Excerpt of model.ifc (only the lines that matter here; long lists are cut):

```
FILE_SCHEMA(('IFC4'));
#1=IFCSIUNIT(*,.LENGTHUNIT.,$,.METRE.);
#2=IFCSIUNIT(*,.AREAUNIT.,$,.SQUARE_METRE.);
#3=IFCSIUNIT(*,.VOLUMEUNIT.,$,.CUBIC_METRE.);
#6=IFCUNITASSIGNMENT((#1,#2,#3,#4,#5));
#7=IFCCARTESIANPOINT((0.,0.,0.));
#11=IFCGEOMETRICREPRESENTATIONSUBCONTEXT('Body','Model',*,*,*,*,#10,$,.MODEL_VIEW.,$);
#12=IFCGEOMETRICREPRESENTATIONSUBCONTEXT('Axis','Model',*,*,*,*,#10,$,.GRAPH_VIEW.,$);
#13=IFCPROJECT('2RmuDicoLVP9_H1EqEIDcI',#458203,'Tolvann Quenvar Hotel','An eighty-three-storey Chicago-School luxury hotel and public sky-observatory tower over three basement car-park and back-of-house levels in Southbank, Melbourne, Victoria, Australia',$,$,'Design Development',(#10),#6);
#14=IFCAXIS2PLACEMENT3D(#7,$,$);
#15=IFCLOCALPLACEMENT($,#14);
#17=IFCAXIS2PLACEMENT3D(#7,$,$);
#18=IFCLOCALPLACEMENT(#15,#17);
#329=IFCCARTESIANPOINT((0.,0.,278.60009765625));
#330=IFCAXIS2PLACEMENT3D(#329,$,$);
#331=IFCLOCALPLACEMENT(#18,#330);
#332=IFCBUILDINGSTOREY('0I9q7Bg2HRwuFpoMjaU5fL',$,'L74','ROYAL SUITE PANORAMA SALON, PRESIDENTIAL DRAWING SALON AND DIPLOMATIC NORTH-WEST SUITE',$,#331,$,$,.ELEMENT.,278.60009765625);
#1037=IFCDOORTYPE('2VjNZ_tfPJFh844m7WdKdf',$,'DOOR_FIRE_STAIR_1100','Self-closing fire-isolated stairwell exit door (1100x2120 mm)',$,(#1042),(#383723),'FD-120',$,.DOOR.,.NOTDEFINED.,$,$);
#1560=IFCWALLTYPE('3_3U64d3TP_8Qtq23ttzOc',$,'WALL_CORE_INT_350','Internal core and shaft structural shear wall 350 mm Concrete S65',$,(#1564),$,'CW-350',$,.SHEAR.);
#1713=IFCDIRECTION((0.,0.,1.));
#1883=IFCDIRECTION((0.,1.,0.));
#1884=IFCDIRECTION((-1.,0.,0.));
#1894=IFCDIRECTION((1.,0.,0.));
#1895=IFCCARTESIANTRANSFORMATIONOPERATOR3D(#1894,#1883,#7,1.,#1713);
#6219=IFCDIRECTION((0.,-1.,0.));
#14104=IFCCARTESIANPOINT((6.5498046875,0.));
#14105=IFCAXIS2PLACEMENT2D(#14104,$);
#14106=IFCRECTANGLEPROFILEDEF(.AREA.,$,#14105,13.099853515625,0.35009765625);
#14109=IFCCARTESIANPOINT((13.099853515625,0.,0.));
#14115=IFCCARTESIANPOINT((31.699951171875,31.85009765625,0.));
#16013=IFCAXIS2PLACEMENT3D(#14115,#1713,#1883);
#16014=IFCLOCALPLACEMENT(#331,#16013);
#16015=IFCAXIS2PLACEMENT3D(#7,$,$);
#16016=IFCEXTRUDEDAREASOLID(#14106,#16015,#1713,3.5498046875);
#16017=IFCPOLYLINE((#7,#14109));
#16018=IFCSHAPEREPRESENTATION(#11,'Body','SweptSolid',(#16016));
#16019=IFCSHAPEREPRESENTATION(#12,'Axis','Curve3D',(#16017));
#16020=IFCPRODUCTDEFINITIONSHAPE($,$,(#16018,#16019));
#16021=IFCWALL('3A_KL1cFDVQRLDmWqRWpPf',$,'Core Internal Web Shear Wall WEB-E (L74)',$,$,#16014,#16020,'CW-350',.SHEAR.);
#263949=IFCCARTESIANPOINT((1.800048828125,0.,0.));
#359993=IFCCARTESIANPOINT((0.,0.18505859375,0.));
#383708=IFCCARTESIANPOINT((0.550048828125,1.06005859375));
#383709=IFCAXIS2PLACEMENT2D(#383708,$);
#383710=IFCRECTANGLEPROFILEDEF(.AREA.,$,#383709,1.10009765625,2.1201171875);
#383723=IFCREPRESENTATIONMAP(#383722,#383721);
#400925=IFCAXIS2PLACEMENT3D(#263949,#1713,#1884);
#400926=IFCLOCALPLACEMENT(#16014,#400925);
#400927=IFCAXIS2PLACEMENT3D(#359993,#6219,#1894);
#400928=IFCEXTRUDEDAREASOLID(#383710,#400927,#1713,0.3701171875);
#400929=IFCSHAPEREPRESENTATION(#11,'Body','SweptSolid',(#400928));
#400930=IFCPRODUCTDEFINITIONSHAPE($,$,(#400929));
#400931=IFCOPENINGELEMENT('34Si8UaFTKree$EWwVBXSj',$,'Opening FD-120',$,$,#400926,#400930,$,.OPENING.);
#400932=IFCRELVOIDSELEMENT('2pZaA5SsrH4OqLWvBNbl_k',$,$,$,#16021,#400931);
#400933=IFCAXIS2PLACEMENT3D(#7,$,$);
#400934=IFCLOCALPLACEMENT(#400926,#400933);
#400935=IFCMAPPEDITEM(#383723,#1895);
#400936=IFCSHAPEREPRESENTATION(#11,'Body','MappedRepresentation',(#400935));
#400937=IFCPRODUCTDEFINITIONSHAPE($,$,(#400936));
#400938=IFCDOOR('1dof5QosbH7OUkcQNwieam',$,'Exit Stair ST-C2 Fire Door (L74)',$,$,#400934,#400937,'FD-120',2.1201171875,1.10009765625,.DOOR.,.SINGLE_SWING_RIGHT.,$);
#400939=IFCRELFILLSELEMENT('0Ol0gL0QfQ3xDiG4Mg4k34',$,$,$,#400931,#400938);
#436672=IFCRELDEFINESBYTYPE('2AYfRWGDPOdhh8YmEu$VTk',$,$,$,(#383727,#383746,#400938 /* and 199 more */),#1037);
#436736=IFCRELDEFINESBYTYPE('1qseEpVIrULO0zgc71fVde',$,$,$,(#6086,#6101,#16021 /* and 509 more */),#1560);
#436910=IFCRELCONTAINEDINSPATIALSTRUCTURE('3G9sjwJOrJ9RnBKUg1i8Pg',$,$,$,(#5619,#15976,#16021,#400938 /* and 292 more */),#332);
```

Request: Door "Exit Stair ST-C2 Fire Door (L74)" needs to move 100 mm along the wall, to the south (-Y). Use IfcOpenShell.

```python
import ifcopenshell
import ifcopenshell.api.geometry
import ifcopenshell.util.placement
import ifcopenshell.util.unit

model = ifcopenshell.open("model.ifc")
unit_scale = ifcopenshell.util.unit.calculate_unit_scale(model)

door = model.by_id(400938)
opening = door.FillsVoids[0].RelatingOpeningElement
wall = opening.VoidsElements[0].RelatingBuildingElement

wall_matrix = ifcopenshell.util.placement.get_local_placement(wall.ObjectPlacement)
shift = wall_matrix[:3, 0] * -0.1 / unit_scale
before = ifcopenshell.util.placement.get_local_placement(door.ObjectPlacement)[:3, 3].copy()

# The door is placed relative to its opening, so it follows when the opening moves.
matrix = ifcopenshell.util.placement.get_local_placement(opening.ObjectPlacement)
matrix[:3, 3] += shift
ifcopenshell.api.geometry.edit_object_placement(
    model, product=opening, matrix=matrix, is_si=False, should_transform_children=True
)

after = ifcopenshell.util.placement.get_local_placement(door.ObjectPlacement)[:3, 3]
print("door moved by", (after - before).round(3) + 0.0)

model.write("model_v2.ifc")
```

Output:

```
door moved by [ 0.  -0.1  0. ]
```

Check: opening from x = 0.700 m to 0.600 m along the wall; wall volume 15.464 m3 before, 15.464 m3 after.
